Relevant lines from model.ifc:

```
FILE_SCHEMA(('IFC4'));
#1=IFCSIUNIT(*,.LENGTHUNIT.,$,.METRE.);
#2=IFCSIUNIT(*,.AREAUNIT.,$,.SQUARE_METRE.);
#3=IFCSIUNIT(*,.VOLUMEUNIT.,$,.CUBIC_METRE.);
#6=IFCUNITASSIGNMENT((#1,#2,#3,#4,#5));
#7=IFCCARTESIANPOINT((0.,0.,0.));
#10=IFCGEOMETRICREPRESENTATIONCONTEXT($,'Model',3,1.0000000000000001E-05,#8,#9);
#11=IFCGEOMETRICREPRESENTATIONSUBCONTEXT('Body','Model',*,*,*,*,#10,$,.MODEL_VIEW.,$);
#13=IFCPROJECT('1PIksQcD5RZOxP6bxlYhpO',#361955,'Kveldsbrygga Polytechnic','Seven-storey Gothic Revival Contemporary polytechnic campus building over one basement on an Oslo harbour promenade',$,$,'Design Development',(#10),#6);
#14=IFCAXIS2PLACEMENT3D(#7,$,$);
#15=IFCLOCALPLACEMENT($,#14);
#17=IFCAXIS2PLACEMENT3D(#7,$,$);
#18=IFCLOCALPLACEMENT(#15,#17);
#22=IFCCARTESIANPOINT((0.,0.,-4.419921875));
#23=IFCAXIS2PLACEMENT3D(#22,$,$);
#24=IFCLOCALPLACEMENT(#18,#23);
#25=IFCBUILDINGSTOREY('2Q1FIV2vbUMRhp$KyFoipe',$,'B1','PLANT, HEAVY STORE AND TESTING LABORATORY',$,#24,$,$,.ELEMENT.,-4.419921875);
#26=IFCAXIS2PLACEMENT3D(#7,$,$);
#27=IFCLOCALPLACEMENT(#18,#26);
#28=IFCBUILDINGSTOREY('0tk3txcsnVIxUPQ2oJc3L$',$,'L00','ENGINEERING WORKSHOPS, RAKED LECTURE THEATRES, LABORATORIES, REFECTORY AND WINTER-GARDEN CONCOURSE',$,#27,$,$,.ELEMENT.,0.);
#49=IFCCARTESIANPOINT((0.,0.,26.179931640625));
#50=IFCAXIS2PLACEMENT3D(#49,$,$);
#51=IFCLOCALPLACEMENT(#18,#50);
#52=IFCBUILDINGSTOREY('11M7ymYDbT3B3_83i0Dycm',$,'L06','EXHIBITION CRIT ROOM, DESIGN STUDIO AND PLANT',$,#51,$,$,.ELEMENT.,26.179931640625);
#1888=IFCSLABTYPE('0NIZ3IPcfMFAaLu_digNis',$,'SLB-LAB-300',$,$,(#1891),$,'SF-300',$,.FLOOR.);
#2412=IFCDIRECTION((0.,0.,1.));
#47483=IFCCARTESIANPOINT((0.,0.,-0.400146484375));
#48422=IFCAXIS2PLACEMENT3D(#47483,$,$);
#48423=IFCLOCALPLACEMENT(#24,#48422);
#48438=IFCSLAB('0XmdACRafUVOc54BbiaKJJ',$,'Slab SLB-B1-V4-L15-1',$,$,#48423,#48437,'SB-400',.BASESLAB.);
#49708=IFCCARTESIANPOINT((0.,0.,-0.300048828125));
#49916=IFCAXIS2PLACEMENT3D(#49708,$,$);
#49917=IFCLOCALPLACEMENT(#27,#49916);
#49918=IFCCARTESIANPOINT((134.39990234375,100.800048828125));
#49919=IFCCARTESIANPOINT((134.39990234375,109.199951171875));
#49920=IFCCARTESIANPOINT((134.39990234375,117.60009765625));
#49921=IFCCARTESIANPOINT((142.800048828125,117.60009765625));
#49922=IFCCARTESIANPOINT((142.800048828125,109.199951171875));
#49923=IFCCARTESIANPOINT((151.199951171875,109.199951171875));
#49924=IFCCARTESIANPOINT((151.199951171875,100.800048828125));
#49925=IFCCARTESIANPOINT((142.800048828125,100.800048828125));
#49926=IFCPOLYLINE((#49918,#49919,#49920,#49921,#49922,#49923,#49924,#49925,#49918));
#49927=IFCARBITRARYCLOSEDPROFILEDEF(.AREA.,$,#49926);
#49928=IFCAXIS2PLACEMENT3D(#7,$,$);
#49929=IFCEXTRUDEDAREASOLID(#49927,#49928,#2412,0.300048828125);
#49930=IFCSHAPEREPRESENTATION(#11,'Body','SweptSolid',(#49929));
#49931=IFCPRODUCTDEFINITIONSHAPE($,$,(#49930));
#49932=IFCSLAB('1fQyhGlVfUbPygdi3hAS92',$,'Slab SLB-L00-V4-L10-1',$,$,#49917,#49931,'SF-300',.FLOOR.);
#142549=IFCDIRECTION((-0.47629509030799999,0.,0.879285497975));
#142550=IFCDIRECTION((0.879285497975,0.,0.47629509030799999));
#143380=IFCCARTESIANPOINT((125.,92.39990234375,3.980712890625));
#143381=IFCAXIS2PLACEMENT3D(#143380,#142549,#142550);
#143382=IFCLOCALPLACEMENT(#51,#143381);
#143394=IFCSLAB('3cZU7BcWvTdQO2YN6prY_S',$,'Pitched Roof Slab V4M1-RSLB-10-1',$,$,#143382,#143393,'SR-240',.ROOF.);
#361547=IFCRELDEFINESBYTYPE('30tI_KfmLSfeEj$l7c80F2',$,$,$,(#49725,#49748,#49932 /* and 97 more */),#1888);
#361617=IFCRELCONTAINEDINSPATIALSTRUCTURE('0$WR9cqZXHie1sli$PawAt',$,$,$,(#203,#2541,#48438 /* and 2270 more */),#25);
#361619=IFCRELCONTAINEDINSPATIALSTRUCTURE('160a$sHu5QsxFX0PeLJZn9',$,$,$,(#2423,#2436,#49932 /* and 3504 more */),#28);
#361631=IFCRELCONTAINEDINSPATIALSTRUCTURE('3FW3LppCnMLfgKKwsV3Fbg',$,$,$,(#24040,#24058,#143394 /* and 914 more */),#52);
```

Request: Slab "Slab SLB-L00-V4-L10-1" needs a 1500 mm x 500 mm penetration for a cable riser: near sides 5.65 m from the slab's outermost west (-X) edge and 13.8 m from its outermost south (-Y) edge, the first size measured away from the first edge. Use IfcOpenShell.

```python
import numpy as np
import ifcopenshell
import ifcopenshell.api.feature
import ifcopenshell.api.geometry
import ifcopenshell.api.root
import ifcopenshell.geom
import ifcopenshell.util.placement
import ifcopenshell.util.representation
import ifcopenshell.util.shape
import ifcopenshell.util.unit

model = ifcopenshell.open("model.ifc")
unit_scale = ifcopenshell.util.unit.calculate_unit_scale(model)
settings = ifcopenshell.geom.settings()


def volume(element):
    """Net volume in cubic metres, openings subtracted."""
    shape = ifcopenshell.geom.create_shape(settings, element)
    return ifcopenshell.util.shape.get_volume(shape.geometry)


slab = model.by_id(49932)
before = volume(slab)

# Extent in the slab's own axes, in metres. The edges named are its -X and -Y sides.
slab_shape = ifcopenshell.geom.create_shape(settings, slab)
vertices = ifcopenshell.util.shape.get_vertices(slab_shape.geometry)
x_min, y_min, bottom = vertices.min(axis=0)
top = vertices[:, 2].max()

opening = ifcopenshell.api.root.create_entity(model, ifc_class="IfcOpeningElement", name="Cable riser opening", predefined_type="OPENING")
context = ifcopenshell.util.representation.get_context(model, "Model", "Body", "MODEL_VIEW")
width, depth = 1.5, 0.5
outline = [(0.0, 0.0), (width, 0.0), (width, depth), (0.0, depth), (0.0, 0.0)]
# Overshoot both faces by 50 mm so the cut is clean.
shape = ifcopenshell.api.geometry.add_slab_representation(
    model, context=context, depth=top - bottom + 0.1, polyline=outline
)
ifcopenshell.api.geometry.assign_representation(model, product=opening, representation=shape)

matrix = ifcopenshell.util.placement.get_local_placement(slab.ObjectPlacement)
matrix[:, 3] = matrix @ np.append(np.array([x_min + 5.65, y_min + 13.8, bottom - 0.05]) / unit_scale, 1.0)
ifcopenshell.api.geometry.edit_object_placement(model, product=opening, matrix=matrix, is_si=False)
ifcopenshell.api.feature.add_feature(model, feature=opening, element=slab)

after = volume(slab)

print(f"slab volume {before:.3f} -> {after:.3f} m3")

model.write("model_edited.ifc")
```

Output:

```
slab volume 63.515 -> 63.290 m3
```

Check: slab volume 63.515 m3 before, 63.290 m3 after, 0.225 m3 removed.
